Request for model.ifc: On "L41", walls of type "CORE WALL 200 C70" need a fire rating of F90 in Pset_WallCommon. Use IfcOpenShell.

First a look at what the model holds.

```python
import ifcopenshell
import ifcopenshell.util.element

model = ifcopenshell.open("model.ifc")
print(model.schema)
storey = next(s for s in model.by_type("IfcBuildingStorey") if s.Name == "L41")
walls = [e for e in ifcopenshell.util.element.get_decomposition(storey) if e.is_a("IfcWall")]
seen = {}
for e in walls:
    element_type = ifcopenshell.util.element.get_type(e)
    key = (element_type.Name if element_type != e and element_type else None, ifcopenshell.util.element.get_pset(e, "Pset_WallCommon", "FireRating"))
    seen[key] = seen.get(key, 0) + 1
for (name, value), count in sorted(seen.items(), key=str):
    print(count, "x", name, "|", value)
```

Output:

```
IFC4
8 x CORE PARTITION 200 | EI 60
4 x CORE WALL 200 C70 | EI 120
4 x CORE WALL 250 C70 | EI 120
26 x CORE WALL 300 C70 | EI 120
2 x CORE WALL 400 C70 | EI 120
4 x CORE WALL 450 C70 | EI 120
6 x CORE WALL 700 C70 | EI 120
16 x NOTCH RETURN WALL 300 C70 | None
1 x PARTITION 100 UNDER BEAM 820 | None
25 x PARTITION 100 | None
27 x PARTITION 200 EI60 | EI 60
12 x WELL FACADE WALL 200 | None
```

```python
import ifcopenshell
import ifcopenshell.api.pset
import ifcopenshell.util.element

model = ifcopenshell.open("model.ifc")

storey = next(s for s in model.by_type("IfcBuildingStorey") if s.Name == "L41")
walls = [e for e in ifcopenshell.util.element.get_decomposition(storey) if e.is_a("IfcWall")]

count = 0
for e in walls:
    element_type = ifcopenshell.util.element.get_type(e)
    if element_type in (None, e) or element_type.Name != "CORE WALL 200 C70":
        continue
    found = ifcopenshell.util.element.get_pset(e, "Pset_WallCommon", should_inherit=False)
    if found:
        pset = model.by_id(found["id"])
        if len(ifcopenshell.util.element.get_elements_by_pset(pset)) > 1:
            pset = ifcopenshell.api.pset.unshare_pset(model, products=[e], pset=pset)[0]
    else:
        pset = ifcopenshell.api.pset.add_pset(model, product=e, name="Pset_WallCommon")
    ifcopenshell.api.pset.edit_pset(model, pset=pset, properties={"FireRating": "F90"})
    count += 1

print(count, "walls updated")

model.write("model_v2.ifc")
```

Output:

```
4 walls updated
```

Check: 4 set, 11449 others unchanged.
